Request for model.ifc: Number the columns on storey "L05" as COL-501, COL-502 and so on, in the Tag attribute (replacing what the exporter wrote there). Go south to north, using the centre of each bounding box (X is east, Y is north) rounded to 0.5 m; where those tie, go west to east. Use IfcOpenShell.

First a look at what the model holds.

```python
import ifcopenshell
import ifcopenshell.util.element
import ifcopenshell.util.placement

model = ifcopenshell.open("model.ifc")
print(model.schema)
storey = next(s for s in model.by_type("IfcBuildingStorey") if s.Name == "L05")
columns = [e for e in ifcopenshell.util.element.get_decomposition(storey) if e.is_a("IfcColumn")]
for e in sorted(columns, key=lambda e: e.id()):
    origin = ifcopenshell.util.placement.get_local_placement(e.ObjectPlacement)[:3, 3]
    print(e.id(), e.Tag, e.Name, origin.round(2) + 0.0, sep=" | ")
```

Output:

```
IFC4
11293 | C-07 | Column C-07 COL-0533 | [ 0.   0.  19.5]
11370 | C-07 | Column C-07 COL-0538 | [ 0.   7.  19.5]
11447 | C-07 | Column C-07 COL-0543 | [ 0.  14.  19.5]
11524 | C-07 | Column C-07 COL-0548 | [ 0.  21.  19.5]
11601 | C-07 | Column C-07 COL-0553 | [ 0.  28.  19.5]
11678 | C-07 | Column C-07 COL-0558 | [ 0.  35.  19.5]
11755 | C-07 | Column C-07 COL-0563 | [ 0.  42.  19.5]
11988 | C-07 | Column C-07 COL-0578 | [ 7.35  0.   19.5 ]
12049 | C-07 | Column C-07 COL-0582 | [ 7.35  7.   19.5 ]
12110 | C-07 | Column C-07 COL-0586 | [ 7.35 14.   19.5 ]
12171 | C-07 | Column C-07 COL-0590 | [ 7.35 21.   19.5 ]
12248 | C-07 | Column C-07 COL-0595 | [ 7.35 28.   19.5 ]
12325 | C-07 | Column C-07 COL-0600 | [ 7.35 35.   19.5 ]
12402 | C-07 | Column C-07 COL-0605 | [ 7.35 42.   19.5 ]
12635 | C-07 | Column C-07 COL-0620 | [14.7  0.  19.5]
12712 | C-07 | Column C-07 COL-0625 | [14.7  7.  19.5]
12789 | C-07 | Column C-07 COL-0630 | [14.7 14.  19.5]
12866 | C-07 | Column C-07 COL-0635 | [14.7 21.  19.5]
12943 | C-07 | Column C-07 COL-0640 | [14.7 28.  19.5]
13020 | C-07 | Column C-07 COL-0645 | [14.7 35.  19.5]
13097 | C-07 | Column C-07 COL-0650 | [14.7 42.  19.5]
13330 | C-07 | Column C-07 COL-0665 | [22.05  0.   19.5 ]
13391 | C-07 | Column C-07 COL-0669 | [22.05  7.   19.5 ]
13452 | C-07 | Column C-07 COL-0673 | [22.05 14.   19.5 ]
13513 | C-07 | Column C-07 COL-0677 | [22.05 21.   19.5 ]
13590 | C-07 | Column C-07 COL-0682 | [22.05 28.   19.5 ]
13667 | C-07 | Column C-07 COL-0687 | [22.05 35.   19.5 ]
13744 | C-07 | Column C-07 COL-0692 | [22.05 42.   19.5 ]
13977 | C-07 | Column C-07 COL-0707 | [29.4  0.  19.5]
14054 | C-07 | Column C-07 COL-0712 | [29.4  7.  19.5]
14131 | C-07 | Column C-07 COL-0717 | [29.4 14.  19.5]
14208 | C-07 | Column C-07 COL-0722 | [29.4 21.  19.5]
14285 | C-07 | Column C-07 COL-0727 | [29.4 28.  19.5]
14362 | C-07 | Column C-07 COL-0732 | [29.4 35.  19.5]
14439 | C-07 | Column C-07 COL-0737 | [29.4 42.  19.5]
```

```python
import ifcopenshell
import ifcopenshell.geom
import ifcopenshell.util.element
import ifcopenshell.util.shape

model = ifcopenshell.open("model.ifc")
settings = ifcopenshell.geom.settings()
settings.set("use-world-coords", True)


def centre(element):
    shape = ifcopenshell.geom.create_shape(settings, element)
    return ifcopenshell.util.shape.get_bbox_centroid(shape.geometry)


storey = next(s for s in model.by_type("IfcBuildingStorey") if s.Name == "L05")
columns = [e for e in ifcopenshell.util.element.get_decomposition(storey) if e.is_a("IfcColumn")]

# Insertion points can sit at a corner or the storey origin, so sort by the geometry (in metres).
centres = {e: centre(e) for e in columns}
columns.sort(key=lambda e: (round(centres[e][1] / 0.5), centres[e][0]))

for i, e in enumerate(columns, start=1):
    number = f"COL-5{i:02d}"
    e.Tag = number
    print(e.id(), number)

model.write("model_v2.ifc")
```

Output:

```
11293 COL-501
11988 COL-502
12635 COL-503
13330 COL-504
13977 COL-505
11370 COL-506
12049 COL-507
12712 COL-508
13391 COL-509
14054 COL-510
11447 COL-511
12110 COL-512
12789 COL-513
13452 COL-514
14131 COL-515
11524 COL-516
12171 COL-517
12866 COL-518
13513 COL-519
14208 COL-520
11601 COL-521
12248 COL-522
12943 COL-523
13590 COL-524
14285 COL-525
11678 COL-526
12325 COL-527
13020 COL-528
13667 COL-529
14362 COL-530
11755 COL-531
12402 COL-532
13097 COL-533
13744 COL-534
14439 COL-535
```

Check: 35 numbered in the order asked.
